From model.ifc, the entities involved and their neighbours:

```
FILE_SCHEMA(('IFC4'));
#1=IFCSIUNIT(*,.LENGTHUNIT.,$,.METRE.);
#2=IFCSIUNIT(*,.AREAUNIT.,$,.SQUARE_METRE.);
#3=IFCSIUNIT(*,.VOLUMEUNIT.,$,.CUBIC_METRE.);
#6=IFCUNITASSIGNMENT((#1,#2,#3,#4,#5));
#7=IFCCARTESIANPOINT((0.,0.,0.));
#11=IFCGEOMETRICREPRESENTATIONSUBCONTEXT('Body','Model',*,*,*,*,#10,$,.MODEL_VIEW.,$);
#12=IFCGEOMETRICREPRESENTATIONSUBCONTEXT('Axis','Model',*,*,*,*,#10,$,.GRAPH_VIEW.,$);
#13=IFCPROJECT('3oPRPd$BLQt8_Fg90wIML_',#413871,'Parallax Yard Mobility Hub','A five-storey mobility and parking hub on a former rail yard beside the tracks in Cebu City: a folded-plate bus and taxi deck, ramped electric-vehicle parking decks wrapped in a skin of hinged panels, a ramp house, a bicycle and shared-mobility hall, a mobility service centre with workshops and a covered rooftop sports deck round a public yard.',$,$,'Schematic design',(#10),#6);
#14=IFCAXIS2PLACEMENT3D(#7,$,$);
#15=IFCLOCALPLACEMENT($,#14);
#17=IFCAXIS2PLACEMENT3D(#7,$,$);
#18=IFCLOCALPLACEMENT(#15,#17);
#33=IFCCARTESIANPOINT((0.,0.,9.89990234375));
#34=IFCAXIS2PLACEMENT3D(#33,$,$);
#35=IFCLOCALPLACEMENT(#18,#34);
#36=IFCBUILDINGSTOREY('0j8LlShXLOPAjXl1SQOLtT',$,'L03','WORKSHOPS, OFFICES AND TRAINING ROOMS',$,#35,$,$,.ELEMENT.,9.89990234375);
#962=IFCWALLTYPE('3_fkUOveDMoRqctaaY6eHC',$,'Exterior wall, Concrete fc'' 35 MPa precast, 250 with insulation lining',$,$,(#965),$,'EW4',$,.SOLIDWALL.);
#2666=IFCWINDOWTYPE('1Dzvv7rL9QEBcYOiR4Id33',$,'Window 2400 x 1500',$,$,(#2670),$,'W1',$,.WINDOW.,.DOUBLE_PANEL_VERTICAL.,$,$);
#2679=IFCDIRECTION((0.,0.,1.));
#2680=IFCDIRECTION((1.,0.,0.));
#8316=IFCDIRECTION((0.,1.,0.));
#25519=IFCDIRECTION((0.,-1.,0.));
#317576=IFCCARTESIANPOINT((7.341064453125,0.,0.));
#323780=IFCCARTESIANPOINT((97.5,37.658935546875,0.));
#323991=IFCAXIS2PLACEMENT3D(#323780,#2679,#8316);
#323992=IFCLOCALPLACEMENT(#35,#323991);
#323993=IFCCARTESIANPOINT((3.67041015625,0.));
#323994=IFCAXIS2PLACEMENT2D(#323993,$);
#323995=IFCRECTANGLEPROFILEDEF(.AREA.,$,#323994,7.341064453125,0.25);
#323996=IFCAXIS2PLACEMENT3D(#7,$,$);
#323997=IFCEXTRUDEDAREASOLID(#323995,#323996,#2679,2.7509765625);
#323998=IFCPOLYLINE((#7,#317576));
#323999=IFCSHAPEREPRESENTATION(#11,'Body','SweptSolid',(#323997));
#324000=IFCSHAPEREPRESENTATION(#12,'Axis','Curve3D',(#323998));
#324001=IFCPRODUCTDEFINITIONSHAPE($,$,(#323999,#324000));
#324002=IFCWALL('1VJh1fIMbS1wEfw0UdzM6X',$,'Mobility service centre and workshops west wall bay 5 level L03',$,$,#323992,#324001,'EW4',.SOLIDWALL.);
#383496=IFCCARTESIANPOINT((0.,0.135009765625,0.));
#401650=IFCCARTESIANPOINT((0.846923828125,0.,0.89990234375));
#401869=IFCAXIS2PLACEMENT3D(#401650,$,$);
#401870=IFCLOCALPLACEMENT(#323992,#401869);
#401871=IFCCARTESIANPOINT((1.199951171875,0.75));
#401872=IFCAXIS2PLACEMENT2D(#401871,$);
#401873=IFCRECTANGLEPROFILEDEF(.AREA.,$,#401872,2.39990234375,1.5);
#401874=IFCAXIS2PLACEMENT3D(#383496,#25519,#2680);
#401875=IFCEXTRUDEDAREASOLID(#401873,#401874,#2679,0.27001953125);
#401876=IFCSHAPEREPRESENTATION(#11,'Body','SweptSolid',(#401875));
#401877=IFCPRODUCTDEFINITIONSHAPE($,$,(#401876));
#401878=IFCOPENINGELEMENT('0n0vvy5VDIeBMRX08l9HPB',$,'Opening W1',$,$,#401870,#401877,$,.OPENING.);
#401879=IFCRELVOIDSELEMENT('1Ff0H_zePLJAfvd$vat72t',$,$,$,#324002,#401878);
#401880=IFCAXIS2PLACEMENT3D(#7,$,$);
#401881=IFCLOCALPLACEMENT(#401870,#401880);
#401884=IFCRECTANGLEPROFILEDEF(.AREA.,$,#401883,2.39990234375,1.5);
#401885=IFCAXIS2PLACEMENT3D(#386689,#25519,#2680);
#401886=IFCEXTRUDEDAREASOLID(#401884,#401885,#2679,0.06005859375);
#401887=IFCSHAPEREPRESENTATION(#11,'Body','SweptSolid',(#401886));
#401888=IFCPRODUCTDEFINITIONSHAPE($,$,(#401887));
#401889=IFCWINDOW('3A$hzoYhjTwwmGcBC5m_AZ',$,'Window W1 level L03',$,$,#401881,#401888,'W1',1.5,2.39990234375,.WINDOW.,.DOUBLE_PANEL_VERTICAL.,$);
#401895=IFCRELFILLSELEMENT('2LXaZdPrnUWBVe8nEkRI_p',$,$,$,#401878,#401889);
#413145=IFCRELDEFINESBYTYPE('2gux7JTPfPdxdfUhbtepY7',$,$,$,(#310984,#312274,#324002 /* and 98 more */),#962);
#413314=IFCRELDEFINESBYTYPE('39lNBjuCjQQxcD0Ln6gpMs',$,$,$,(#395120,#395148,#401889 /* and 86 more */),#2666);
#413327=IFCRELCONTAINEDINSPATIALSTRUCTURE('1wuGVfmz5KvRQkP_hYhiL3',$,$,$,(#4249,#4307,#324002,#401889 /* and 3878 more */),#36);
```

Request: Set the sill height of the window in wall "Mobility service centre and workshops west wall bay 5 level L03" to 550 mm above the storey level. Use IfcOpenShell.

```python
import numpy as np
import ifcopenshell
import ifcopenshell.api.geometry
import ifcopenshell.geom
import ifcopenshell.util.element
import ifcopenshell.util.placement
import ifcopenshell.util.shape
import ifcopenshell.util.unit

model = ifcopenshell.open("model.ifc")
unit_scale = ifcopenshell.util.unit.calculate_unit_scale(model)

window = model.by_guid("3A$hzoYhjTwwmGcBC5m_AZ")
opening = window.FillsVoids[0].RelatingOpeningElement
storey = ifcopenshell.util.element.get_container(window, ifc_class="IfcBuildingStorey")
level = ifcopenshell.util.placement.get_local_placement(storey.ObjectPlacement)[2, 3]

# The opening's origin need not be at the sill, so measure its lowest point.
shape = ifcopenshell.geom.create_shape(ifcopenshell.geom.settings(), opening)
bottom = ifcopenshell.util.shape.get_shape_bottom_elevation(shape, shape.geometry) / unit_scale
dz = level + 0.55 / unit_scale - bottom

shift = np.array([0.0, 0.0, dz])
# The window is placed relative to its opening, so it follows when the opening moves.
matrix = ifcopenshell.util.placement.get_local_placement(opening.ObjectPlacement)
matrix[:3, 3] += shift
ifcopenshell.api.geometry.edit_object_placement(
    model, product=opening, matrix=matrix, is_si=False, should_transform_children=True
)

print(f"moved by {dz * unit_scale:+.3f} m")

model.write("model_v2.ifc")
```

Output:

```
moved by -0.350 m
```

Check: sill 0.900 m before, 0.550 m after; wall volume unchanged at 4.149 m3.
